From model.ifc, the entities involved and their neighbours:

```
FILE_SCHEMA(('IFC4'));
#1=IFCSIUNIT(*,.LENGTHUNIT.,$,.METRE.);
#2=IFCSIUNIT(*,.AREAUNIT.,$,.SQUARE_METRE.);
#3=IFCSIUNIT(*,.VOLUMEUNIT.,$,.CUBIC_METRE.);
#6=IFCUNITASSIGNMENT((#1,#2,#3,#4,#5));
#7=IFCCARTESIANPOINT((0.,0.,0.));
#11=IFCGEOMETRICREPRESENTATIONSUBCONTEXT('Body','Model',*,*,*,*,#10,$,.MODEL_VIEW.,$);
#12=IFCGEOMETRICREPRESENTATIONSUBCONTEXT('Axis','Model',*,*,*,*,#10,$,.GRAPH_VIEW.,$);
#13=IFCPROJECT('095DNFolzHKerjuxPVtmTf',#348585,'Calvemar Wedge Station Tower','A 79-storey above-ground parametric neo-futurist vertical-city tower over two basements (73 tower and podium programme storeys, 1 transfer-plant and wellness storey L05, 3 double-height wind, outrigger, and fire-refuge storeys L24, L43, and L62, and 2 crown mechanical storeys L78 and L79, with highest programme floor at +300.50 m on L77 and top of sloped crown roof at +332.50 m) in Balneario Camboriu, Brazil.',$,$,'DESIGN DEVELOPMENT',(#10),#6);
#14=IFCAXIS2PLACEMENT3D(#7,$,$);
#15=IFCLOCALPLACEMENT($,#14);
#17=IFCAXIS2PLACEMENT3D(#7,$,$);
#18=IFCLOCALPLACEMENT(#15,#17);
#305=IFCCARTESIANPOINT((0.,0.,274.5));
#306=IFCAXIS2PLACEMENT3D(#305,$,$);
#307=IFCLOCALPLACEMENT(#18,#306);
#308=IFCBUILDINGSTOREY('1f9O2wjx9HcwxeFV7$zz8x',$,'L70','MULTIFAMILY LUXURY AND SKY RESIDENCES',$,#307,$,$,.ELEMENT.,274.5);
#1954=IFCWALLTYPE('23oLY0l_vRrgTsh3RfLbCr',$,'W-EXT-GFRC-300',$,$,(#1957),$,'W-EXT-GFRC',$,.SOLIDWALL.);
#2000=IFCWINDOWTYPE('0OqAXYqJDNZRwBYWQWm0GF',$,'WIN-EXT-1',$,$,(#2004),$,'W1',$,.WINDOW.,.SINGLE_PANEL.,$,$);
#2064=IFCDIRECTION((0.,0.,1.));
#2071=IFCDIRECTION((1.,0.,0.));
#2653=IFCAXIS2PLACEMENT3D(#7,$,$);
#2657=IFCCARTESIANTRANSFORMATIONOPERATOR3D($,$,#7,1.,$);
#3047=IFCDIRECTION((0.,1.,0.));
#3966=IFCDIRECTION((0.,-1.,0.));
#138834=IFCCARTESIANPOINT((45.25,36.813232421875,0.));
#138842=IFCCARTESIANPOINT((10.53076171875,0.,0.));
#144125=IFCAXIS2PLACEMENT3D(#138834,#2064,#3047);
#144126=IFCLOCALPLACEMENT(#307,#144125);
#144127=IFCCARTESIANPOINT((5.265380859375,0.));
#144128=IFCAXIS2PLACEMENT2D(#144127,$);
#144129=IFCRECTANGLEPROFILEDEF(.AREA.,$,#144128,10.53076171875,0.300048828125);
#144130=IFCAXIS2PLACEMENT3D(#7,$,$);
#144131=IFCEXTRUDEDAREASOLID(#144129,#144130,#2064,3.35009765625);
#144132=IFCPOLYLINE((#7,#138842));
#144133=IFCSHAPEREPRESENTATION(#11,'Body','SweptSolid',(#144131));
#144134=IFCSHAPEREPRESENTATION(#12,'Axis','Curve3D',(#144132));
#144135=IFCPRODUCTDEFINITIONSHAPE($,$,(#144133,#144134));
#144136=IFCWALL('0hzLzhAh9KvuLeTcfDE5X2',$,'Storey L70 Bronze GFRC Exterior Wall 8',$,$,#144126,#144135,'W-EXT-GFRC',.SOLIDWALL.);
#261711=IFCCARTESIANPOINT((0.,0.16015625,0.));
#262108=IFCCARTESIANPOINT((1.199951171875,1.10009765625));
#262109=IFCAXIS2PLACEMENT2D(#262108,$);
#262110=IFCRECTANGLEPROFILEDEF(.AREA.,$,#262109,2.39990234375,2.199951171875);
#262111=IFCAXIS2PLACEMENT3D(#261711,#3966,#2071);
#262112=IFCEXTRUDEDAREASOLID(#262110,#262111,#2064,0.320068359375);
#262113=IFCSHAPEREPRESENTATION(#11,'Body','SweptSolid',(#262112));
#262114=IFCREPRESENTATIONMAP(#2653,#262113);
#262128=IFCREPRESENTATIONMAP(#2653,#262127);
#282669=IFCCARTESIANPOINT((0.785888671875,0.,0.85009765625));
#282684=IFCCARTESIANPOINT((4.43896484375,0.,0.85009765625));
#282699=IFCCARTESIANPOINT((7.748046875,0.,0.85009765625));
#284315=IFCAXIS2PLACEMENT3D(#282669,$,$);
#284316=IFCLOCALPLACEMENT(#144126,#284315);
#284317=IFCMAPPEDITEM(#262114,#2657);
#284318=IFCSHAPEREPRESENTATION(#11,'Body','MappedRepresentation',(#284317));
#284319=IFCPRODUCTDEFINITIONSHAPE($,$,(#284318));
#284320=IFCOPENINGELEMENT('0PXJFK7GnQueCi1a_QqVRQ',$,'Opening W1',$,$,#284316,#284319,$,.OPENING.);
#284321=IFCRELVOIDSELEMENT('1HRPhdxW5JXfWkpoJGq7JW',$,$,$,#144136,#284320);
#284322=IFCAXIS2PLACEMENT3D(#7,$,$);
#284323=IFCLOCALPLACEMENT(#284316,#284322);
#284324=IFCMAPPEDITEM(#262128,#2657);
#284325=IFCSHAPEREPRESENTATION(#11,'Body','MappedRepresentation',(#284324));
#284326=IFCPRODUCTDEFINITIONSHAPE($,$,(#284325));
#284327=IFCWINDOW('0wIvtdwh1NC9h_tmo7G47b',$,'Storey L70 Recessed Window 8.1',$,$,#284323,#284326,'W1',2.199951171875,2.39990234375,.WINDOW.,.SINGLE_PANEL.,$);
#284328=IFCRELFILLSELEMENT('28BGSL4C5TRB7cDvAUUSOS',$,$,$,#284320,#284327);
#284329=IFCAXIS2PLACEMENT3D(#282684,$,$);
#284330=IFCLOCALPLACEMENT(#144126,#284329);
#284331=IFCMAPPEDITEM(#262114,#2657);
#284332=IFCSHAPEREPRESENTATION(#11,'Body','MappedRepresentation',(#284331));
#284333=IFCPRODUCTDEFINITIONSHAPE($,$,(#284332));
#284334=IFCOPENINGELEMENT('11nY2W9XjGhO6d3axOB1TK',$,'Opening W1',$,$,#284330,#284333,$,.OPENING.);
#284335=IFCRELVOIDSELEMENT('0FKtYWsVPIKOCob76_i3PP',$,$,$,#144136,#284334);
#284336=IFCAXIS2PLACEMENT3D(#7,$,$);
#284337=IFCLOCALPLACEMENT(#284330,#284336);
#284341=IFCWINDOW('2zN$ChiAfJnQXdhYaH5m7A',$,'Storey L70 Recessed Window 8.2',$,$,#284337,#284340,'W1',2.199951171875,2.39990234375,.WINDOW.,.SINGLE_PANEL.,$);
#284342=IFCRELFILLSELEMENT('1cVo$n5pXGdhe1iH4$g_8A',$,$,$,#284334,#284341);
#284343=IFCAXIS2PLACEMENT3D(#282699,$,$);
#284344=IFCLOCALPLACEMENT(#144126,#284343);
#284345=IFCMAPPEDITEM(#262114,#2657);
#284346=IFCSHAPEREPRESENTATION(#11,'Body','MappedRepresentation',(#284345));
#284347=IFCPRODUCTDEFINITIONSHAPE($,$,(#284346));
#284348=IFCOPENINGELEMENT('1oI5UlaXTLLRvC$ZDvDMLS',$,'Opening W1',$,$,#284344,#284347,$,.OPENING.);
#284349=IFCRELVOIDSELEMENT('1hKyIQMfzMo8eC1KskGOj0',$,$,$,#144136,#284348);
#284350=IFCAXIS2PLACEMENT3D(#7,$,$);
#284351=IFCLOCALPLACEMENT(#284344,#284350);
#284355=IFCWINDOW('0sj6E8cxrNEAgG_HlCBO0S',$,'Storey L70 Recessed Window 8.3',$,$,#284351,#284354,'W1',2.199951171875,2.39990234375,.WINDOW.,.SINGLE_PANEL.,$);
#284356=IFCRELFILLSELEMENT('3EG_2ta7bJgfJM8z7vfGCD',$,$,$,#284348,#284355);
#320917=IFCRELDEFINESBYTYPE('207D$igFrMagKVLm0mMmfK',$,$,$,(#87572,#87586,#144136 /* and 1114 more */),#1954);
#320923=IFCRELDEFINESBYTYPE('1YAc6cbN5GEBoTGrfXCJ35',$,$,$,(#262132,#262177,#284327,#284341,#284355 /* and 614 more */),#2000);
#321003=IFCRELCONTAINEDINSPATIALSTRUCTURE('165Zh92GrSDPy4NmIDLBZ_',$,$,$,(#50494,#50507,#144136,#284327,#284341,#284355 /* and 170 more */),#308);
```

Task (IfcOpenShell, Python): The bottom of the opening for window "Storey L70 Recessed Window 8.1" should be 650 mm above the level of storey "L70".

```python
import numpy as np
import ifcopenshell
import ifcopenshell.api.geometry
import ifcopenshell.geom
import ifcopenshell.util.element
import ifcopenshell.util.placement
import ifcopenshell.util.shape
import ifcopenshell.util.unit

model = ifcopenshell.open("model.ifc")
unit_scale = ifcopenshell.util.unit.calculate_unit_scale(model)

window = model.by_guid("0wIvtdwh1NC9h_tmo7G47b")
opening = window.FillsVoids[0].RelatingOpeningElement
storey = ifcopenshell.util.element.get_container(window, ifc_class="IfcBuildingStorey")
level = ifcopenshell.util.placement.get_local_placement(storey.ObjectPlacement)[2, 3]

# The opening's origin need not be at the sill, so measure its lowest point.
shape = ifcopenshell.geom.create_shape(ifcopenshell.geom.settings(), opening)
bottom = ifcopenshell.util.shape.get_shape_bottom_elevation(shape, shape.geometry) / unit_scale
dz = level + 0.65 / unit_scale - bottom

shift = np.array([0.0, 0.0, dz])
# The window is placed relative to its opening, so it follows when the opening moves.
matrix = ifcopenshell.util.placement.get_local_placement(opening.ObjectPlacement)
matrix[:3, 3] += shift
ifcopenshell.api.geometry.edit_object_placement(
    model, product=opening, matrix=matrix, is_si=False, should_transform_children=True
)

print(f"moved by {dz * unit_scale:+.3f} m")

model.write("model_rev.ifc")
```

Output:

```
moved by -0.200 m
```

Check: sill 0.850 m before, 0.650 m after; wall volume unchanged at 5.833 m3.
